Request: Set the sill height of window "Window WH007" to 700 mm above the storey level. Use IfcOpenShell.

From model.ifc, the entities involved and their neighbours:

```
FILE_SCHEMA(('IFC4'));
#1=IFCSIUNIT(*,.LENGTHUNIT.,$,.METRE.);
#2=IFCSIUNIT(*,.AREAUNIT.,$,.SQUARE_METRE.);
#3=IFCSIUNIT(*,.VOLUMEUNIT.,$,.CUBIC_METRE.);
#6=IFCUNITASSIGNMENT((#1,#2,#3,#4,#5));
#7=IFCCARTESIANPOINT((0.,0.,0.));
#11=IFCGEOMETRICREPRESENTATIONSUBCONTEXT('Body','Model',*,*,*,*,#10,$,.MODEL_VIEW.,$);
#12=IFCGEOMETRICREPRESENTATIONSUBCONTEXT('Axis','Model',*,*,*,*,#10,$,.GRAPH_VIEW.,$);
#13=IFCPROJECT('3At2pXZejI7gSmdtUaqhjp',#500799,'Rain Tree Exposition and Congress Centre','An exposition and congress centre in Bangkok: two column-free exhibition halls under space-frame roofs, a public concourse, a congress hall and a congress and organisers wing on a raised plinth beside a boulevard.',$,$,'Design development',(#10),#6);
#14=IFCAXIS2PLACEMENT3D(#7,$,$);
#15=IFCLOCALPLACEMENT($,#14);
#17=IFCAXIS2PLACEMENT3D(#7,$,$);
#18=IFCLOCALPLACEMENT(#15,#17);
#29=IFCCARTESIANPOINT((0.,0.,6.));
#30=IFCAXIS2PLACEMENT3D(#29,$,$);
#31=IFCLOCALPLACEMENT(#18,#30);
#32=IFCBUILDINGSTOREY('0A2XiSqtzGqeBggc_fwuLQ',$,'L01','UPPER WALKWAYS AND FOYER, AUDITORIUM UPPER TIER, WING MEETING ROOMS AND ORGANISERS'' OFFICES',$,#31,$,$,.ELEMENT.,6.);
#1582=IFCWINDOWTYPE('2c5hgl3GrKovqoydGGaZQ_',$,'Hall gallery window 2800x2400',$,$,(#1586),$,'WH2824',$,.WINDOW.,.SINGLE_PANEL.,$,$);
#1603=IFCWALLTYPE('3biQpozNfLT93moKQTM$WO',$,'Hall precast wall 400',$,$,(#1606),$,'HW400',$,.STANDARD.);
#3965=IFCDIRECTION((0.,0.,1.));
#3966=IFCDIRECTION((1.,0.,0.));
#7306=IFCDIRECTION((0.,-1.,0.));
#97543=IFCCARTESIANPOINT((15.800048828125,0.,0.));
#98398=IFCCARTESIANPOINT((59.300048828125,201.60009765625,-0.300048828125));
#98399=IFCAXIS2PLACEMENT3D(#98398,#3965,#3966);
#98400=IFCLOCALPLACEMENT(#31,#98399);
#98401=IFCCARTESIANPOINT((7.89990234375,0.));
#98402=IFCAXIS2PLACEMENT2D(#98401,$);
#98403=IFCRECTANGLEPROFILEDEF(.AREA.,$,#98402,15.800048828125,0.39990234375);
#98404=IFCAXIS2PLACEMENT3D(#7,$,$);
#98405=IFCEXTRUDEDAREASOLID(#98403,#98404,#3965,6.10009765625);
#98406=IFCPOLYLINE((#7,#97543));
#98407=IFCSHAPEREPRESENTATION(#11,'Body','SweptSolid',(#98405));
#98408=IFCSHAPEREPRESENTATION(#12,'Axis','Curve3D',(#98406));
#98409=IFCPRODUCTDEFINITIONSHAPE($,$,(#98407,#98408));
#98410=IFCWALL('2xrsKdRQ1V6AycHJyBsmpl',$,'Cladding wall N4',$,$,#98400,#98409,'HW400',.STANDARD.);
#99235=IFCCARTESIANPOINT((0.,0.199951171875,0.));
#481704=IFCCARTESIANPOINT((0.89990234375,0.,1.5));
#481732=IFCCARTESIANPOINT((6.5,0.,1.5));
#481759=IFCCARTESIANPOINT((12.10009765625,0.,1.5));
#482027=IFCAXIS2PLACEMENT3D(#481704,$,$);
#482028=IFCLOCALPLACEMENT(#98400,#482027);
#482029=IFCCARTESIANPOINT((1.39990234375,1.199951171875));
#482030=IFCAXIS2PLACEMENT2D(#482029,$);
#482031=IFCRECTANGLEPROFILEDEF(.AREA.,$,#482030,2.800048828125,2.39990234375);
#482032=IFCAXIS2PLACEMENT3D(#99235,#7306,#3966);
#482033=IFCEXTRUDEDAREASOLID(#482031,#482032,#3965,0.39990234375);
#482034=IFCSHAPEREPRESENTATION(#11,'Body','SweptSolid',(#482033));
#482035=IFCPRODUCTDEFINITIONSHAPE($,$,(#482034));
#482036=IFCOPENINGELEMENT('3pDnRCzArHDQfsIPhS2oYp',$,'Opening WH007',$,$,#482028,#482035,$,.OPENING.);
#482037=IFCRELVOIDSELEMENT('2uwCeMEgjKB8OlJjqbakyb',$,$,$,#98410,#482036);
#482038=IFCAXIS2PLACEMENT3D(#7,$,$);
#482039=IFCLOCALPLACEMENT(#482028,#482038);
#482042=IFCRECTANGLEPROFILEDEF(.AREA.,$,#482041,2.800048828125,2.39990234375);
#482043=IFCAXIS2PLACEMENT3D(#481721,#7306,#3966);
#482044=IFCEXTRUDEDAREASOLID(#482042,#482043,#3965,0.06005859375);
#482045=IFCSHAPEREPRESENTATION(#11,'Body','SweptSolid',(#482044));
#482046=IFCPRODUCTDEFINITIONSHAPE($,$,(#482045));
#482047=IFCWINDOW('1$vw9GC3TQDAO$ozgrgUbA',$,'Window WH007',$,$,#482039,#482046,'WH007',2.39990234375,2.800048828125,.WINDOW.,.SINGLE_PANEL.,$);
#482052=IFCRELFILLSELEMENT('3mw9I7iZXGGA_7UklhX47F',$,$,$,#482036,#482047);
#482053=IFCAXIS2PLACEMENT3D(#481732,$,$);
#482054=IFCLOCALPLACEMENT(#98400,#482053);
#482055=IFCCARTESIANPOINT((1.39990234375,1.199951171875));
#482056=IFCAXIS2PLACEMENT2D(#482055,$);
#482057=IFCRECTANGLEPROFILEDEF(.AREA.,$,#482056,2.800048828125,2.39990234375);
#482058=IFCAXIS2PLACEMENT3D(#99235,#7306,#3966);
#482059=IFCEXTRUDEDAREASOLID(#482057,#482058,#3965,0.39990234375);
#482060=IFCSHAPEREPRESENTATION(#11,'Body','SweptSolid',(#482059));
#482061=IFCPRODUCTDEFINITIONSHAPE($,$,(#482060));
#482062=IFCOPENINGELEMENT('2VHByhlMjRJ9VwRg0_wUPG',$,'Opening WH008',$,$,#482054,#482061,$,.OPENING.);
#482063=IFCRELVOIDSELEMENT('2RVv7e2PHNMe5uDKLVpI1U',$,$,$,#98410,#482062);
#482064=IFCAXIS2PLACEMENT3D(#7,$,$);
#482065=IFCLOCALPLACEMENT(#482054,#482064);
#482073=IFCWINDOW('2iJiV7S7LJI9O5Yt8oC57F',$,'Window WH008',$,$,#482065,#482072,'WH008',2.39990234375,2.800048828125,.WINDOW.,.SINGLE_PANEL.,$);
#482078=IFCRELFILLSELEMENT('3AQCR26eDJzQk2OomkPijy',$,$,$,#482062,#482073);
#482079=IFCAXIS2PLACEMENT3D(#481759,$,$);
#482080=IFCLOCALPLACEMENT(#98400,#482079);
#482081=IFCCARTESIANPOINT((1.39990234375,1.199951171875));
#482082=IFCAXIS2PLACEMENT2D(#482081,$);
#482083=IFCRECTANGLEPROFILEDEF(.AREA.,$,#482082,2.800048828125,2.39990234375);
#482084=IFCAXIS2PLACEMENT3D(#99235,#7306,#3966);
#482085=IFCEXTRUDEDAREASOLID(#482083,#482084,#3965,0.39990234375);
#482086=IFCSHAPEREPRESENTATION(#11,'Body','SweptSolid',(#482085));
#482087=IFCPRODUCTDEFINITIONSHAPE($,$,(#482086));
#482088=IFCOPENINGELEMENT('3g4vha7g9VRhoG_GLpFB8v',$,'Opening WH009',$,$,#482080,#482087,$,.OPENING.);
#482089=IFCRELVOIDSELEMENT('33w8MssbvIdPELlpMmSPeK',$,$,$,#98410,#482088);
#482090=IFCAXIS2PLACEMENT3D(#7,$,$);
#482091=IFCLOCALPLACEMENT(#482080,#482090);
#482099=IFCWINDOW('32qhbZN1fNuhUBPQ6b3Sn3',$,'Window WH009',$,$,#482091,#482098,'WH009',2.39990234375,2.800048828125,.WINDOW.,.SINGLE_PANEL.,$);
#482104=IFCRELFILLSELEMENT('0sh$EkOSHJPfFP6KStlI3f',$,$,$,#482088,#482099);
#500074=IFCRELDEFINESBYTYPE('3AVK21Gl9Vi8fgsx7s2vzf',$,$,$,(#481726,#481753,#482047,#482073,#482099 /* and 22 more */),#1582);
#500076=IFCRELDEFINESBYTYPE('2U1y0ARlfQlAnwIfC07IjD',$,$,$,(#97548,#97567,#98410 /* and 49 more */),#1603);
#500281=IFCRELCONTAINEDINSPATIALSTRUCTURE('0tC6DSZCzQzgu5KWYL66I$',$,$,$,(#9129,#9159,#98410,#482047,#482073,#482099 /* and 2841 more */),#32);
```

```python
import numpy as np
import ifcopenshell
import ifcopenshell.api.geometry
import ifcopenshell.geom
import ifcopenshell.util.element
import ifcopenshell.util.placement
import ifcopenshell.util.shape
import ifcopenshell.util.unit

model = ifcopenshell.open("model.ifc")
unit_scale = ifcopenshell.util.unit.calculate_unit_scale(model)

window = model.by_id(482047)
opening = window.FillsVoids[0].RelatingOpeningElement
storey = ifcopenshell.util.element.get_container(window, ifc_class="IfcBuildingStorey")
level = ifcopenshell.util.placement.get_local_placement(storey.ObjectPlacement)[2, 3]

# The opening's origin need not be at the sill, so measure its lowest point.
shape = ifcopenshell.geom.create_shape(ifcopenshell.geom.settings(), opening)
bottom = ifcopenshell.util.shape.get_shape_bottom_elevation(shape, shape.geometry) / unit_scale
dz = level + 0.7 / unit_scale - bottom

shift = np.array([0.0, 0.0, dz])
# The window is placed relative to its opening, so it follows when the opening moves.
matrix = ifcopenshell.util.placement.get_local_placement(opening.ObjectPlacement)
matrix[:3, 3] += shift
ifcopenshell.api.geometry.edit_object_placement(
    model, product=opening, matrix=matrix, is_si=False, should_transform_children=True
)

print(f"moved by {dz * unit_scale:+.3f} m")

model.write("model_updated.ifc")
```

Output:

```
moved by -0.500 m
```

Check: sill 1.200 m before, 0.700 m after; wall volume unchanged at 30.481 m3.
